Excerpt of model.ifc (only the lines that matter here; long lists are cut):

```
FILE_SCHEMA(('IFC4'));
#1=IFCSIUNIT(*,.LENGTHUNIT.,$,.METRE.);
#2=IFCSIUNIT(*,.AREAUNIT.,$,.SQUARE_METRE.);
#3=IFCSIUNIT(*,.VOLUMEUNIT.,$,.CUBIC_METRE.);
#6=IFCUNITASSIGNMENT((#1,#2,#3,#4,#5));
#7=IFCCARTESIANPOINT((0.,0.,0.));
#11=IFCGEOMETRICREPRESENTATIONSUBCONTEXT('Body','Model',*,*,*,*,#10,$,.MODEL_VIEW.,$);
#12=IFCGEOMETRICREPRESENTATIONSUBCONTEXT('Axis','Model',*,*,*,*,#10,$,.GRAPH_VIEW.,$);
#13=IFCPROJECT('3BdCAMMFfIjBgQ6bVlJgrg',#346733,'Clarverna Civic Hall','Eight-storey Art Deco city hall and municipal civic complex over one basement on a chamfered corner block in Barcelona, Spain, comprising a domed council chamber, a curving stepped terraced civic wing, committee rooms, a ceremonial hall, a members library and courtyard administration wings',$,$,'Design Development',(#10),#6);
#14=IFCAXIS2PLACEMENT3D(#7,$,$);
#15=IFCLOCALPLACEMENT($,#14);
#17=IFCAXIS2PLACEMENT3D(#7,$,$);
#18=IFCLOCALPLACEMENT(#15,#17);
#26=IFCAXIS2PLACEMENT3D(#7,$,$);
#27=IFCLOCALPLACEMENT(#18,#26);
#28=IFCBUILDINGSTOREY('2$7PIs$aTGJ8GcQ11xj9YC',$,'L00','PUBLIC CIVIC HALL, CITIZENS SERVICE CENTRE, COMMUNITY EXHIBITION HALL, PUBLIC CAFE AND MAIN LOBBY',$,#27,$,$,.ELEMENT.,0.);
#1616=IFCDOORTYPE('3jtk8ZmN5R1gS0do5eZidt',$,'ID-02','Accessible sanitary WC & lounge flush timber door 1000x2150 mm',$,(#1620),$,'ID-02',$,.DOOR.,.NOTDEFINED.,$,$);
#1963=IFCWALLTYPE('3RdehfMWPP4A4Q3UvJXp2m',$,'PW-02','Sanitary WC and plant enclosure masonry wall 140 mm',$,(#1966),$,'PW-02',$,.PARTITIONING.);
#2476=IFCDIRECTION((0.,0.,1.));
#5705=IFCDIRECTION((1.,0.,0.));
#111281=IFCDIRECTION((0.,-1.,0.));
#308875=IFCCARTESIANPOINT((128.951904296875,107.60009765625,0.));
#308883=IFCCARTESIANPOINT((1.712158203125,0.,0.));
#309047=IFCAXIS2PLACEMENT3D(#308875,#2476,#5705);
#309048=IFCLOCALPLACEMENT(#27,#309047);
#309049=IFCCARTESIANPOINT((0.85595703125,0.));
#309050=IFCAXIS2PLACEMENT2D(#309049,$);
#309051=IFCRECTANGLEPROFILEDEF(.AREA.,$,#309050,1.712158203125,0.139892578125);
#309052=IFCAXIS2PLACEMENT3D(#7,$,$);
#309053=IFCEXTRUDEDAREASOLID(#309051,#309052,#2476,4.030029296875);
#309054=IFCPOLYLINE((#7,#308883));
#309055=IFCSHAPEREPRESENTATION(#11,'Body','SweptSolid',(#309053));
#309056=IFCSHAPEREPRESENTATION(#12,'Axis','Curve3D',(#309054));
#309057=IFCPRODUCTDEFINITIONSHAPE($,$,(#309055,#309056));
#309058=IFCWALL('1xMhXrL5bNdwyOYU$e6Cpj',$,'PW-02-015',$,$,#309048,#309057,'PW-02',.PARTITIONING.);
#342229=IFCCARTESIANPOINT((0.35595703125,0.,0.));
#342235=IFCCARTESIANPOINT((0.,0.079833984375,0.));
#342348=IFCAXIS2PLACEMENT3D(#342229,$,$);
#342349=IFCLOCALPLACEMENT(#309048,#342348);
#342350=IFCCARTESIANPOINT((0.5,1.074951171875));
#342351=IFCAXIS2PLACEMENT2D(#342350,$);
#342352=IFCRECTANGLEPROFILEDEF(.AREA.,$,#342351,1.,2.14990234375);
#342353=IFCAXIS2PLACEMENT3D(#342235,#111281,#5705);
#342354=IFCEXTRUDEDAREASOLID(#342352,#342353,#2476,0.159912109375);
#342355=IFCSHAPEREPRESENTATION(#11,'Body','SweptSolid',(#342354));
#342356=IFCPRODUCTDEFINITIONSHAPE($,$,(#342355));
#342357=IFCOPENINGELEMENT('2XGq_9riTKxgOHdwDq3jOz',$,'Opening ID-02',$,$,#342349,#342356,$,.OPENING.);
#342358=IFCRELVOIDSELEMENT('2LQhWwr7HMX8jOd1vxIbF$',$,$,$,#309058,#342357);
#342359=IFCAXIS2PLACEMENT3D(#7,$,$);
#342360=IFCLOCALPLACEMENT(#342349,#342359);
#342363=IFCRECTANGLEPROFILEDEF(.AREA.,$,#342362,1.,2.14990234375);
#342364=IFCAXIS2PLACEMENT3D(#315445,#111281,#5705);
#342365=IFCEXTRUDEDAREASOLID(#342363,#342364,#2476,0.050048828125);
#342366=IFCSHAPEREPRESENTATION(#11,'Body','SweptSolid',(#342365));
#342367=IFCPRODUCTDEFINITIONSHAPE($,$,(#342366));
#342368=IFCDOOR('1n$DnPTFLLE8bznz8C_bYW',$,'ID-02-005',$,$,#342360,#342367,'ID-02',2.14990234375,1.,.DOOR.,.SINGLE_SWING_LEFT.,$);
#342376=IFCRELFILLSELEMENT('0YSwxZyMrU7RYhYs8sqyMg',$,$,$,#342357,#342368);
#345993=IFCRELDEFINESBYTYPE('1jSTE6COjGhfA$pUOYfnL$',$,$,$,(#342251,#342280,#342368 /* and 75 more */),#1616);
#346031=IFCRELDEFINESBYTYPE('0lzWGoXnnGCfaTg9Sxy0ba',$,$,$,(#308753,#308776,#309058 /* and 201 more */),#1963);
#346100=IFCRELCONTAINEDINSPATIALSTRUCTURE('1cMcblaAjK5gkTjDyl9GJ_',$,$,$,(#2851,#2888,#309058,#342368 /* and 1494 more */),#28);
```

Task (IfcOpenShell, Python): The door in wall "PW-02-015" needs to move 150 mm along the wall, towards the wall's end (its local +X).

```python
import ifcopenshell
import ifcopenshell.api.geometry
import ifcopenshell.util.placement

model = ifcopenshell.open("model.ifc")

door = model.by_guid("1n$DnPTFLLE8bznz8C_bYW")
opening = door.FillsVoids[0].RelatingOpeningElement
wall = opening.VoidsElements[0].RelatingBuildingElement

wall_matrix = ifcopenshell.util.placement.get_local_placement(wall.ObjectPlacement)
shift = wall_matrix[:3, 0] * 0.15
before = ifcopenshell.util.placement.get_local_placement(door.ObjectPlacement)[:3, 3].copy()

# The door is placed relative to its opening, so it follows when the opening moves.
matrix = ifcopenshell.util.placement.get_local_placement(opening.ObjectPlacement)
matrix[:3, 3] += shift
ifcopenshell.api.geometry.edit_object_placement(
    model, product=opening, matrix=matrix, is_si=False, should_transform_children=True
)

after = ifcopenshell.util.placement.get_local_placement(door.ObjectPlacement)[:3, 3]
print("door moved by", (after - before).round(3) + 0.0)

model.write("model_v2.ifc")
```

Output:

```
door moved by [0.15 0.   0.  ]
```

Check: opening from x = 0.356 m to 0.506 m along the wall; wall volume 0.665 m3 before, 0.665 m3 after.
